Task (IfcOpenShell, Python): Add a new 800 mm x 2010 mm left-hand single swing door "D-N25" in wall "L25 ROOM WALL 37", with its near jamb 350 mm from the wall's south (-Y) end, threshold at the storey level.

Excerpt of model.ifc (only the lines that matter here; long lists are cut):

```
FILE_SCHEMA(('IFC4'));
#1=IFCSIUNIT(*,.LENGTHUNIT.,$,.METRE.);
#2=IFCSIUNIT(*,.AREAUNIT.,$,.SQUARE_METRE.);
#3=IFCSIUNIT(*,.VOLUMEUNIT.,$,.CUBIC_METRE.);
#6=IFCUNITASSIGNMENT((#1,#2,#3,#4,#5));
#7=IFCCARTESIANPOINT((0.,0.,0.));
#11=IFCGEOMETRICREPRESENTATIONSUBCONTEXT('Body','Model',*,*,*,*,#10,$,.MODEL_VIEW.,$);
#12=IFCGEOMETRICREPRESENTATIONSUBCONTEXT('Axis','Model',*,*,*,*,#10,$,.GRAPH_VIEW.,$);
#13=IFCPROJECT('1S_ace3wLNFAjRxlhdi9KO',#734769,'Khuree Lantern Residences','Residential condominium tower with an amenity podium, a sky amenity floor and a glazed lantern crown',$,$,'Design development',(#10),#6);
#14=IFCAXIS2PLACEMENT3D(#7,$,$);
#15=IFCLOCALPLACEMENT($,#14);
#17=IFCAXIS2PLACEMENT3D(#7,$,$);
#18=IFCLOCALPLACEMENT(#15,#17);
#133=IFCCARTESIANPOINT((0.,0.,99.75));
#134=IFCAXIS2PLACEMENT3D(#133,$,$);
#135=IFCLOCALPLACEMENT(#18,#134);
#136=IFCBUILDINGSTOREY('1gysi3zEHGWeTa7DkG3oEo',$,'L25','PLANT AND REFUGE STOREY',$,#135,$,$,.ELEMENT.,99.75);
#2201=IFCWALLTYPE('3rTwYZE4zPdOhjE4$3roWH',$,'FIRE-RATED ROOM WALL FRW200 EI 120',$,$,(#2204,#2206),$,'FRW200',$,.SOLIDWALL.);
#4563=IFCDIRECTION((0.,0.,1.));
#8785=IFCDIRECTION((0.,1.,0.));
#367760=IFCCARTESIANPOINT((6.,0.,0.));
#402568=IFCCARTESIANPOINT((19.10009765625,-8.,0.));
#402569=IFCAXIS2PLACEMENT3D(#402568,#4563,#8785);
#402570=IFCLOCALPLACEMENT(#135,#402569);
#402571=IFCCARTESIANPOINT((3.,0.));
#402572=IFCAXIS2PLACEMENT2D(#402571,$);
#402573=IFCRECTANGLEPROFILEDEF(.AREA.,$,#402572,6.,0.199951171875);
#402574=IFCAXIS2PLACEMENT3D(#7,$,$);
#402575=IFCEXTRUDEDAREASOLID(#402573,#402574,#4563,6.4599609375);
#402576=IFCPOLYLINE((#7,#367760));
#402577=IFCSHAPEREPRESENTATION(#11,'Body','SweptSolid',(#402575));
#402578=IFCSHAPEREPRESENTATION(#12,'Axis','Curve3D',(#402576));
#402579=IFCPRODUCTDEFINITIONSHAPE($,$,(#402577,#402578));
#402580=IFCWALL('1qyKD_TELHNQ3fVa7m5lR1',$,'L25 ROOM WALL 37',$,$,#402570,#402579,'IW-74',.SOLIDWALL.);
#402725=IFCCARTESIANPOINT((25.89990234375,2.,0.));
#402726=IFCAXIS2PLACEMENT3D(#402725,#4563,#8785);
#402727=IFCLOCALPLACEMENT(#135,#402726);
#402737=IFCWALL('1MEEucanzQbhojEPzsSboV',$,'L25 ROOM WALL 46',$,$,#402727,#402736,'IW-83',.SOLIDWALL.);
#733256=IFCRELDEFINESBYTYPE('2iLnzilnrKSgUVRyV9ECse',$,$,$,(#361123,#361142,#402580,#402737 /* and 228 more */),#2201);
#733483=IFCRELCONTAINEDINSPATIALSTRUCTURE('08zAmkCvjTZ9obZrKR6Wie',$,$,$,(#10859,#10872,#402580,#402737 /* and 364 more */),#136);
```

```python
import numpy as np
import ifcopenshell
import ifcopenshell.api.feature
import ifcopenshell.api.geometry
import ifcopenshell.api.root
import ifcopenshell.api.spatial
import ifcopenshell.geom
import ifcopenshell.util.element
import ifcopenshell.util.placement
import ifcopenshell.util.representation
import ifcopenshell.util.shape
import ifcopenshell.util.unit

model = ifcopenshell.open("model.ifc")
unit_scale = ifcopenshell.util.unit.calculate_unit_scale(model)
settings = ifcopenshell.geom.settings()


def volume(element):
    """Net volume in cubic metres, openings subtracted."""
    shape = ifcopenshell.geom.create_shape(settings, element)
    return ifcopenshell.util.shape.get_volume(shape.geometry)


wall = model.by_guid("1qyKD_TELHNQ3fVa7m5lR1")
storey = ifcopenshell.util.element.get_container(wall, ifc_class="IfcBuildingStorey")
context = ifcopenshell.util.representation.get_context(model, "Model", "Body", "MODEL_VIEW")
before = volume(wall)

width, height, from_end, sill = 0.8, 2.01, 0.35, 0.0  # metres

# The wall runs along its own X axis, and the end named is its -X end.
wall_shape = ifcopenshell.geom.create_shape(settings, wall)
x, y, z = ifcopenshell.util.shape.get_vertices(wall_shape.geometry).T
start = x.min() + from_end
face, thickness = float(y.min()), float(y.max() - y.min())
wall_matrix = ifcopenshell.util.placement.get_local_placement(wall.ObjectPlacement)
level = ifcopenshell.util.placement.get_local_placement(storey.ObjectPlacement)[2, 3]


def in_wall(x, y):
    """Placement at x, y metres in the wall's axes, at sill height."""
    matrix = wall_matrix.copy()
    matrix[:, 3] = wall_matrix @ np.array([x / unit_scale, y / unit_scale, 0.0, 1.0])
    matrix[2, 3] = level + sill / unit_scale
    return matrix


# Opening: a box that overshoots both wall faces by 50 mm.
opening = ifcopenshell.api.root.create_entity(model, ifc_class="IfcOpeningElement", predefined_type="OPENING")
box = ifcopenshell.api.geometry.add_wall_representation(
    model, context=context, length=width, height=height, thickness=thickness + 0.1
)
ifcopenshell.api.geometry.assign_representation(model, product=opening, representation=box)
ifcopenshell.api.geometry.edit_object_placement(model, product=opening, matrix=in_wall(start, face - 0.05), is_si=False)
ifcopenshell.api.feature.add_feature(model, feature=opening, element=wall)

door = ifcopenshell.api.root.create_entity(model, ifc_class="IfcDoor", name="D-N25", predefined_type="DOOR")
door.OverallWidth, door.OverallHeight = width / unit_scale, height / unit_scale
door.OperationType = "SINGLE_SWING_LEFT"
body = ifcopenshell.api.geometry.add_door_representation(
    model,
    context=context,
    overall_width=door.OverallWidth,
    overall_height=door.OverallHeight,
    operation_type="SINGLE_SWING_LEFT",
    lining_properties={"LiningDepth": thickness / unit_scale, "ThresholdDepth": thickness / unit_scale},
)
ifcopenshell.api.geometry.assign_representation(model, product=door, representation=body)
ifcopenshell.api.spatial.assign_container(model, products=[door], relating_structure=storey)
ifcopenshell.api.feature.add_filling(model, opening=opening, element=door)

# The lining spans the wall, so the door starts at the wall face.
ifcopenshell.api.geometry.edit_object_placement(model, product=door, matrix=in_wall(start, face), is_si=False)

after = volume(wall)

print(f"wall volume {before:.3f} -> {after:.3f} m3")

model.write("model_edited.ifc")
```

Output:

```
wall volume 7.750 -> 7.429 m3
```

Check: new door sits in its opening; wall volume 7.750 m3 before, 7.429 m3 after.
